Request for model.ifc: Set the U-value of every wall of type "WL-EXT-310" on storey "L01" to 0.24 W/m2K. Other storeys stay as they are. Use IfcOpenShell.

First a look at what the model holds.

```python
import ifcopenshell
import ifcopenshell.util.element

model = ifcopenshell.open("model.ifc")
print(model.schema)
storey = next(s for s in model.by_type("IfcBuildingStorey") if s.Name == "L01")
walls = [e for e in ifcopenshell.util.element.get_decomposition(storey) if e.is_a("IfcWall")]
seen = {}
for e in walls:
    element_type = ifcopenshell.util.element.get_type(e)
    key = (element_type.Name if element_type != e and element_type else None, ifcopenshell.util.element.get_pset(e, "Pset_WallCommon", "ThermalTransmittance"))
    seen[key] = seen.get(key, 0) + 1
for (name, value), count in sorted(seen.items(), key=str):
    print(count, "x", name, "|", value)
```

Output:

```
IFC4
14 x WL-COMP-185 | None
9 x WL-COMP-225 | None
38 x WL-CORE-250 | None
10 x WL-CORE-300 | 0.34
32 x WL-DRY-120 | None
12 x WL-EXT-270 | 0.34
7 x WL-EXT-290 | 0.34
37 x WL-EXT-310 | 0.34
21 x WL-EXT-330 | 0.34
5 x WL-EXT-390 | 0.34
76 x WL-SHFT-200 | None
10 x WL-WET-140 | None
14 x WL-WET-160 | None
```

```python
import ifcopenshell
import ifcopenshell.api.pset
import ifcopenshell.util.element

model = ifcopenshell.open("model.ifc")

storey = next(s for s in model.by_type("IfcBuildingStorey") if s.Name == "L01")
walls = [e for e in ifcopenshell.util.element.get_decomposition(storey) if e.is_a("IfcWall")]

count = 0
for e in walls:
    element_type = ifcopenshell.util.element.get_type(e)
    if element_type in (None, e) or element_type.Name != "WL-EXT-310":
        continue
    # add_pset returns the element's existing set when there is one.
    pset = ifcopenshell.api.pset.add_pset(model, product=e, name="Pset_WallCommon")
    ifcopenshell.api.pset.edit_pset(model, pset=pset, properties={"ThermalTransmittance": 0.24})
    count += 1

print(count, "walls updated")

model.write("model_updated.ifc")
```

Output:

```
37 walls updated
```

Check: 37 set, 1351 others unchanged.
